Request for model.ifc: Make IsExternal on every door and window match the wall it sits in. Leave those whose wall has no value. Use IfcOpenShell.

First a look at what the model holds.

```python
import ifcopenshell
import ifcopenshell.util.element

model = ifcopenshell.open("model.ifc")
print(model.schema)
seen = {}
for e in model.by_type("IfcDoor") + model.by_type("IfcWindow"):
    if not e.FillsVoids:
        continue
    host = e.FillsVoids[0].RelatingOpeningElement.VoidsElements[0].RelatingBuildingElement
    own = ifcopenshell.util.element.get_pset(e, f"Pset_{e.is_a()[3:].removesuffix('StandardCase')}Common", "IsExternal")
    wall = ifcopenshell.util.element.get_pset(host, "Pset_WallCommon", "IsExternal")
    seen[e.is_a(), own, wall] = seen.get((e.is_a(), own, wall), 0) + 1
for (cls, own, wall), count in sorted(seen.items(), key=str):
    print(count, cls, "IsExternal:", own, "| host wall:", wall)
```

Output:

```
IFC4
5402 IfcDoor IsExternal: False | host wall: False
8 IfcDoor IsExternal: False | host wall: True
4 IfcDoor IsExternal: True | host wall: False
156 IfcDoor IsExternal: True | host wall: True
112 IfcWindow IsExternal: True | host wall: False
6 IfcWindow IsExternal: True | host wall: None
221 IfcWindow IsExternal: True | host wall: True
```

```python
import ifcopenshell
import ifcopenshell.api.pset
import ifcopenshell.util.element

model = ifcopenshell.open("model.ifc")

count = 0
for ifc_class, pset_name in (("IfcDoor", "Pset_DoorCommon"), ("IfcWindow", "Pset_WindowCommon")):
    for e in model.by_type(ifc_class):
        if not e.FillsVoids:
            continue
        host = e.FillsVoids[0].RelatingOpeningElement.VoidsElements[0].RelatingBuildingElement
        external = ifcopenshell.util.element.get_pset(host, "Pset_WallCommon", "IsExternal")
        if external is None or ifcopenshell.util.element.get_pset(e, pset_name, "IsExternal") == external:
            continue
        found = ifcopenshell.util.element.get_pset(e, pset_name, should_inherit=False)
        if found:
            pset = model.by_id(found["id"])
            if len(ifcopenshell.util.element.get_elements_by_pset(pset)) > 1:
                pset = ifcopenshell.api.pset.unshare_pset(model, products=[e], pset=pset)[0]
        else:
            pset = ifcopenshell.api.pset.add_pset(model, product=e, name=pset_name)
        ifcopenshell.api.pset.edit_pset(model, pset=pset, properties={"IsExternal": external})
        count += 1

print(count, "updated")

model.write("model-out.ifc")
```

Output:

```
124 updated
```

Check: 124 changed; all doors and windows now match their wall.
